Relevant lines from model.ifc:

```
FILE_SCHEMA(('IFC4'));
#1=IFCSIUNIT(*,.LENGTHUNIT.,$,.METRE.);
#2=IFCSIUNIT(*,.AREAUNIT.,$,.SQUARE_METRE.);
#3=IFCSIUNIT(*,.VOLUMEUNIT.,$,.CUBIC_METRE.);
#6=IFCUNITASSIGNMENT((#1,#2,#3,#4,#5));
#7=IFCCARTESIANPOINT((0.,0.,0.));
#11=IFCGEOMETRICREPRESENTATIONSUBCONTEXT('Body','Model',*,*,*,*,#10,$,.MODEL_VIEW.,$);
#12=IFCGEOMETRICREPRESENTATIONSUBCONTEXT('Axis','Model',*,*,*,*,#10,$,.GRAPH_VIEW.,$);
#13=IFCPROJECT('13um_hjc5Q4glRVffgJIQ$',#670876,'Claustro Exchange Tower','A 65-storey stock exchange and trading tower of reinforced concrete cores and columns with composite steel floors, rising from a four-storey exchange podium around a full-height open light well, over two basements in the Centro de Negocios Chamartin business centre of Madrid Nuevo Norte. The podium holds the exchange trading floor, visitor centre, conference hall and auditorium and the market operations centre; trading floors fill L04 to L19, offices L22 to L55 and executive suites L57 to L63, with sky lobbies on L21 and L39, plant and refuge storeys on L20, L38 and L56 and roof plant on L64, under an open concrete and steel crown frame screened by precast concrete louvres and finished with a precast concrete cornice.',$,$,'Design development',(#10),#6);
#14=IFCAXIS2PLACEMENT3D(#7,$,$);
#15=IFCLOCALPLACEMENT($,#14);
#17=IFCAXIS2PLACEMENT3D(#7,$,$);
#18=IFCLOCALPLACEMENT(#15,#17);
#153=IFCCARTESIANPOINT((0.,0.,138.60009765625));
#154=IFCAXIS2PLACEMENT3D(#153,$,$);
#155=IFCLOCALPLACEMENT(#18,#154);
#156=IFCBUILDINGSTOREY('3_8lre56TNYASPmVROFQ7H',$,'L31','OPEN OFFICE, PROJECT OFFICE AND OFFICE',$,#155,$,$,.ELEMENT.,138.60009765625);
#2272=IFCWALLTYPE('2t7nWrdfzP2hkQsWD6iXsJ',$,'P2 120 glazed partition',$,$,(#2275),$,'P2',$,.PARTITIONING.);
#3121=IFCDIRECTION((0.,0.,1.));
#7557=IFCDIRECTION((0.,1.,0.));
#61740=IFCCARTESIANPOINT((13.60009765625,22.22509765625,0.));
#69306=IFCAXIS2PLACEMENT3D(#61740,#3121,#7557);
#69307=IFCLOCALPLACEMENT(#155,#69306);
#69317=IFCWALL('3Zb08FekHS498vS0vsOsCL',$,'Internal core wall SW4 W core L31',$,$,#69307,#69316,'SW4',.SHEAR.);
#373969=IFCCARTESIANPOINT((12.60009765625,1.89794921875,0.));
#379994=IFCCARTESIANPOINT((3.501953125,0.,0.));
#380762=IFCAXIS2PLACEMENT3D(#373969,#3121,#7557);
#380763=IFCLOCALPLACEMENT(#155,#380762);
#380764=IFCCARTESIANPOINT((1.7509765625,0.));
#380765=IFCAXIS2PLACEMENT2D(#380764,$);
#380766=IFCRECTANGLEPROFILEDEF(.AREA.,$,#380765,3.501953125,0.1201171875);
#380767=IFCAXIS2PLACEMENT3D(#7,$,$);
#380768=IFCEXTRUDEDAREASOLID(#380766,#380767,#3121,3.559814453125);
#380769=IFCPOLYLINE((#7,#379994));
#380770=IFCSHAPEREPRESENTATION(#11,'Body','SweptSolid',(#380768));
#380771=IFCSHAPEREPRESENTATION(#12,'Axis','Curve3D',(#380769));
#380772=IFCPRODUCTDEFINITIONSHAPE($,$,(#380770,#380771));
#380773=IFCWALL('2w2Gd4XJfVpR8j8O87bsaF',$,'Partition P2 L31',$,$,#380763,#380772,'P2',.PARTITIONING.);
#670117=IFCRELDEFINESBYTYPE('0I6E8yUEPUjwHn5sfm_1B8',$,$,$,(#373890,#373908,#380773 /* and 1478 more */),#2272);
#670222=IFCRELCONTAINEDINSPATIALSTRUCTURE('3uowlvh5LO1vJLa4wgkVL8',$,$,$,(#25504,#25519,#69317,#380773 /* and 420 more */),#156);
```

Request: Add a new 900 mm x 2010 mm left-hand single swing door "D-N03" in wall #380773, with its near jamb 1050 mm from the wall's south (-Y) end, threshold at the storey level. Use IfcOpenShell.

```python
import numpy as np
import ifcopenshell
import ifcopenshell.api.feature
import ifcopenshell.api.geometry
import ifcopenshell.api.root
import ifcopenshell.api.spatial
import ifcopenshell.geom
import ifcopenshell.util.element
import ifcopenshell.util.placement
import ifcopenshell.util.representation
import ifcopenshell.util.shape
import ifcopenshell.util.unit

model = ifcopenshell.open("model.ifc")
unit_scale = ifcopenshell.util.unit.calculate_unit_scale(model)
settings = ifcopenshell.geom.settings()


def volume(element):
    """Net volume in cubic metres, openings subtracted."""
    shape = ifcopenshell.geom.create_shape(settings, element)
    return ifcopenshell.util.shape.get_volume(shape.geometry)


wall = model.by_id(380773)
storey = ifcopenshell.util.element.get_container(wall, ifc_class="IfcBuildingStorey")
context = ifcopenshell.util.representation.get_context(model, "Model", "Body", "MODEL_VIEW")
before = volume(wall)

width, height, from_end, sill = 0.9, 2.01, 1.05, 0.0  # metres

# The wall runs along its own X axis, and the end named is its -X end.
wall_shape = ifcopenshell.geom.create_shape(settings, wall)
x, y, z = ifcopenshell.util.shape.get_vertices(wall_shape.geometry).T
start = x.min() + from_end
face, thickness = float(y.min()), float(y.max() - y.min())
wall_matrix = ifcopenshell.util.placement.get_local_placement(wall.ObjectPlacement)
level = ifcopenshell.util.placement.get_local_placement(storey.ObjectPlacement)[2, 3]


def in_wall(x, y):
    """Placement at x, y metres in the wall's axes, at sill height."""
    matrix = wall_matrix.copy()
    matrix[:, 3] = wall_matrix @ np.array([x / unit_scale, y / unit_scale, 0.0, 1.0])
    matrix[2, 3] = level + sill / unit_scale
    return matrix


# Opening: a box that overshoots both wall faces by 50 mm.
opening = ifcopenshell.api.root.create_entity(model, ifc_class="IfcOpeningElement", predefined_type="OPENING")
box = ifcopenshell.api.geometry.add_wall_representation(
    model, context=context, length=width, height=height, thickness=thickness + 0.1
)
ifcopenshell.api.geometry.assign_representation(model, product=opening, representation=box)
ifcopenshell.api.geometry.edit_object_placement(model, product=opening, matrix=in_wall(start, face - 0.05), is_si=False)
ifcopenshell.api.feature.add_feature(model, feature=opening, element=wall)

door = ifcopenshell.api.root.create_entity(model, ifc_class="IfcDoor", name="D-N03", predefined_type="DOOR")
door.OverallWidth, door.OverallHeight = width / unit_scale, height / unit_scale
door.OperationType = "SINGLE_SWING_LEFT"
body = ifcopenshell.api.geometry.add_door_representation(
    model,
    context=context,
    overall_width=door.OverallWidth,
    overall_height=door.OverallHeight,
    operation_type="SINGLE_SWING_LEFT",
    lining_properties={"LiningDepth": thickness / unit_scale, "ThresholdDepth": thickness / unit_scale},
)
ifcopenshell.api.geometry.assign_representation(model, product=door, representation=body)
ifcopenshell.api.spatial.assign_container(model, products=[door], relating_structure=storey)
ifcopenshell.api.feature.add_filling(model, opening=opening, element=door)

# The lining spans the wall, so the door starts at the wall face.
ifcopenshell.api.geometry.edit_object_placement(model, product=door, matrix=in_wall(start, face), is_si=False)

after = volume(wall)

print(f"wall volume {before:.3f} -> {after:.3f} m3")

model.write("model_updated.ifc")
```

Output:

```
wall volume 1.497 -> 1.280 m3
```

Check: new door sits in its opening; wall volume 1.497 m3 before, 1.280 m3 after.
